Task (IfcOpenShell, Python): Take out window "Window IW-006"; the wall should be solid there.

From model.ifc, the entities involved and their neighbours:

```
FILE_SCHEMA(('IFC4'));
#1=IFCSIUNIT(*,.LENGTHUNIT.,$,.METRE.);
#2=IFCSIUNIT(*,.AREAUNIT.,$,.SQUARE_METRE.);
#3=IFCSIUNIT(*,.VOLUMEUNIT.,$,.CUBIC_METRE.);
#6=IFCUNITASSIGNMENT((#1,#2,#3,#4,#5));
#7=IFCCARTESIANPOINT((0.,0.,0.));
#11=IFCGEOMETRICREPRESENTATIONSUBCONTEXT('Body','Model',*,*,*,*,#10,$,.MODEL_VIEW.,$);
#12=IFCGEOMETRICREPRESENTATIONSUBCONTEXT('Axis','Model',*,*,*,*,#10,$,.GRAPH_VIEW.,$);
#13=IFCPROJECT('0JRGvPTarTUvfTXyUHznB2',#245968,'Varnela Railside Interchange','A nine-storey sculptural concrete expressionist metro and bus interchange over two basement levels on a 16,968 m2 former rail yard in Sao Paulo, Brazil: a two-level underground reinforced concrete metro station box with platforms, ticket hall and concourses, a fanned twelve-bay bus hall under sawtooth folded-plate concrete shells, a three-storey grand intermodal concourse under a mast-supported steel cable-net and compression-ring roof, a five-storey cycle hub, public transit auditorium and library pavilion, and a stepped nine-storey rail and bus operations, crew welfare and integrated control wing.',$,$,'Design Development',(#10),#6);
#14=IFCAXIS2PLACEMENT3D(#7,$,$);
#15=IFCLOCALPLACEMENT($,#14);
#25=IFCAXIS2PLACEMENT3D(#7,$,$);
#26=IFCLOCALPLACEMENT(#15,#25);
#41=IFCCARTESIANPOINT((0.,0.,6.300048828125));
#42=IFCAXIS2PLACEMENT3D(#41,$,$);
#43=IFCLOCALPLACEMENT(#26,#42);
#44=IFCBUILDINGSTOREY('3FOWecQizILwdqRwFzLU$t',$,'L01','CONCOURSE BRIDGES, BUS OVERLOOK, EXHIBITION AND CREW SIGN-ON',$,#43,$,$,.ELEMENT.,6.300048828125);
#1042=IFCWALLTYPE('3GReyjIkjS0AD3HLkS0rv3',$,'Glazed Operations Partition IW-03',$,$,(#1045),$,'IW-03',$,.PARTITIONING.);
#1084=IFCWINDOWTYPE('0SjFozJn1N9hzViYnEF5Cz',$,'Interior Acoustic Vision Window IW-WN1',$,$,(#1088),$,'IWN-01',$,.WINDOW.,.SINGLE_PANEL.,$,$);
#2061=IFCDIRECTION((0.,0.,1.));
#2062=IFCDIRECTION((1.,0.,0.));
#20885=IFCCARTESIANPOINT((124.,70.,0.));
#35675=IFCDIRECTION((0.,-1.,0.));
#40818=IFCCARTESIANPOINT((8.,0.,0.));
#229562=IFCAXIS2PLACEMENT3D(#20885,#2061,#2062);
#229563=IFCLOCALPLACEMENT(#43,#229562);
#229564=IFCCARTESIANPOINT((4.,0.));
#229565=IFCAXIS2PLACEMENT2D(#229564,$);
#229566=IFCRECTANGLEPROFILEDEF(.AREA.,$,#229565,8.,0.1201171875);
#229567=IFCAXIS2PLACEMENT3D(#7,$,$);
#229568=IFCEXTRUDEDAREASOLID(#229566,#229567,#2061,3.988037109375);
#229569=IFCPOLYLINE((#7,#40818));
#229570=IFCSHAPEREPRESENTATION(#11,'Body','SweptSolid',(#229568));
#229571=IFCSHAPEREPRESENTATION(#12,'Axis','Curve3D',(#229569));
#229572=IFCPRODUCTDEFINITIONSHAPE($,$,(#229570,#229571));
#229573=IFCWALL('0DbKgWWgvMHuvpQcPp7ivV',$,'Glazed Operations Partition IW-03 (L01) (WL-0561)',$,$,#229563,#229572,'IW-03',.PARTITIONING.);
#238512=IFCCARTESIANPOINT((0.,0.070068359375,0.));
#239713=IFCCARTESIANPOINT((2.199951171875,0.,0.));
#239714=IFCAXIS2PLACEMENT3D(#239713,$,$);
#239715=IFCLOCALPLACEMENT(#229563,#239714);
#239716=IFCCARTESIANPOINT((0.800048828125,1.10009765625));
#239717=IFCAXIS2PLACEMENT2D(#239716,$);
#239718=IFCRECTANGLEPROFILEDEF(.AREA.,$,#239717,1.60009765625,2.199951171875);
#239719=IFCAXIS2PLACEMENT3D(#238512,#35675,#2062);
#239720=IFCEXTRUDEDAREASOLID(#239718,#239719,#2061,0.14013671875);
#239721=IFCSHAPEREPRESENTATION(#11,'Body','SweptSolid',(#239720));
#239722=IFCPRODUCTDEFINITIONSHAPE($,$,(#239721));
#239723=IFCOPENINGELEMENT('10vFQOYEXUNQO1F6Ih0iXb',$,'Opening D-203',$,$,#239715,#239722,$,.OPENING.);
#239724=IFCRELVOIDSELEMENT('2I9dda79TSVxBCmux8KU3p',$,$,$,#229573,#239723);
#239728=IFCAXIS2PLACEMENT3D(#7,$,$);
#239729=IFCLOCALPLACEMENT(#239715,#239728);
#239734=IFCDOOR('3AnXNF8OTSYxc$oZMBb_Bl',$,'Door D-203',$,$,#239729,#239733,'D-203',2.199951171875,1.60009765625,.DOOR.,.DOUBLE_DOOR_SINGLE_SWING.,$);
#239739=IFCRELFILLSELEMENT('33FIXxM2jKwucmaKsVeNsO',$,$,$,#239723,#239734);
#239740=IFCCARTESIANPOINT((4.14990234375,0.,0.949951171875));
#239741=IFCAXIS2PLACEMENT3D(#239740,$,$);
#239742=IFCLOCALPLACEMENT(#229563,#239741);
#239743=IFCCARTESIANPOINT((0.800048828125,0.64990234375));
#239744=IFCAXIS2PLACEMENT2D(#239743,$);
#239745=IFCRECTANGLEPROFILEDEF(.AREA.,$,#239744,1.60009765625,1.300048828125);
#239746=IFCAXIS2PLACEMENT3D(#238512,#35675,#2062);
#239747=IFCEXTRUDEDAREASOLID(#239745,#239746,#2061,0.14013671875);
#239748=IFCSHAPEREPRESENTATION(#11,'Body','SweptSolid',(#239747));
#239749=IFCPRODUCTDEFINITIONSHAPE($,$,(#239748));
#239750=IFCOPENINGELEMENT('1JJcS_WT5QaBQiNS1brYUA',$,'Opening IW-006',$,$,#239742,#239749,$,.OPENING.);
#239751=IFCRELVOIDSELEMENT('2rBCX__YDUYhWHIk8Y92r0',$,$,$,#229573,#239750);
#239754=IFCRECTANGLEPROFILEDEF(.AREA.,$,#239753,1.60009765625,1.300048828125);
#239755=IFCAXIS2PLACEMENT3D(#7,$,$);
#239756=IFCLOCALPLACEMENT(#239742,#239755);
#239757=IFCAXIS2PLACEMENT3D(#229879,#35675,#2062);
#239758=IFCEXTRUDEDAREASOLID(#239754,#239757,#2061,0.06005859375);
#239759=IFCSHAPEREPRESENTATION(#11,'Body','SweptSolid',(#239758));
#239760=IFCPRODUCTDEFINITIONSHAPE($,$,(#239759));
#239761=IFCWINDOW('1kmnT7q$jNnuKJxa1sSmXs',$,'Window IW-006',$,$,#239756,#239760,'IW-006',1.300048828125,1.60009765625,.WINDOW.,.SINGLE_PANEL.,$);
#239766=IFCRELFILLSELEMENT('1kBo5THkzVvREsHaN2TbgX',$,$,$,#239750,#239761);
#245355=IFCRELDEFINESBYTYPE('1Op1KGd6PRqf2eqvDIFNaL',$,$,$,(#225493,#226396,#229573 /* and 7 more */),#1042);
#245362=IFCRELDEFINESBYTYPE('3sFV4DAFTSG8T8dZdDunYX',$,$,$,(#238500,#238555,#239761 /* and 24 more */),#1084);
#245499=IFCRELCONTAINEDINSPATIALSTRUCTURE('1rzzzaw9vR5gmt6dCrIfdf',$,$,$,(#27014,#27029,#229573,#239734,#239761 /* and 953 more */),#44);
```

```python
import ifcopenshell
import ifcopenshell.api.feature
import ifcopenshell.api.root
import ifcopenshell.geom
import ifcopenshell.util.shape

model = ifcopenshell.open("model.ifc")
settings = ifcopenshell.geom.settings()


def volume(element):
    """Net volume in cubic metres, openings subtracted."""
    shape = ifcopenshell.geom.create_shape(settings, element)
    return ifcopenshell.util.shape.get_volume(shape.geometry)


window = model.by_id(239761)
opening = window.FillsVoids[0].RelatingOpeningElement
wall = opening.VoidsElements[0].RelatingBuildingElement
before = volume(wall)

ifcopenshell.api.root.remove_product(model, product=window)
ifcopenshell.api.feature.remove_feature(model, feature=opening)

after = volume(wall)

print(f"wall volume {before:.3f} -> {after:.3f} m3")

model.write("model_updated.ifc")
```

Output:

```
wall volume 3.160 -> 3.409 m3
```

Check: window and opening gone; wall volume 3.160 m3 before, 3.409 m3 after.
